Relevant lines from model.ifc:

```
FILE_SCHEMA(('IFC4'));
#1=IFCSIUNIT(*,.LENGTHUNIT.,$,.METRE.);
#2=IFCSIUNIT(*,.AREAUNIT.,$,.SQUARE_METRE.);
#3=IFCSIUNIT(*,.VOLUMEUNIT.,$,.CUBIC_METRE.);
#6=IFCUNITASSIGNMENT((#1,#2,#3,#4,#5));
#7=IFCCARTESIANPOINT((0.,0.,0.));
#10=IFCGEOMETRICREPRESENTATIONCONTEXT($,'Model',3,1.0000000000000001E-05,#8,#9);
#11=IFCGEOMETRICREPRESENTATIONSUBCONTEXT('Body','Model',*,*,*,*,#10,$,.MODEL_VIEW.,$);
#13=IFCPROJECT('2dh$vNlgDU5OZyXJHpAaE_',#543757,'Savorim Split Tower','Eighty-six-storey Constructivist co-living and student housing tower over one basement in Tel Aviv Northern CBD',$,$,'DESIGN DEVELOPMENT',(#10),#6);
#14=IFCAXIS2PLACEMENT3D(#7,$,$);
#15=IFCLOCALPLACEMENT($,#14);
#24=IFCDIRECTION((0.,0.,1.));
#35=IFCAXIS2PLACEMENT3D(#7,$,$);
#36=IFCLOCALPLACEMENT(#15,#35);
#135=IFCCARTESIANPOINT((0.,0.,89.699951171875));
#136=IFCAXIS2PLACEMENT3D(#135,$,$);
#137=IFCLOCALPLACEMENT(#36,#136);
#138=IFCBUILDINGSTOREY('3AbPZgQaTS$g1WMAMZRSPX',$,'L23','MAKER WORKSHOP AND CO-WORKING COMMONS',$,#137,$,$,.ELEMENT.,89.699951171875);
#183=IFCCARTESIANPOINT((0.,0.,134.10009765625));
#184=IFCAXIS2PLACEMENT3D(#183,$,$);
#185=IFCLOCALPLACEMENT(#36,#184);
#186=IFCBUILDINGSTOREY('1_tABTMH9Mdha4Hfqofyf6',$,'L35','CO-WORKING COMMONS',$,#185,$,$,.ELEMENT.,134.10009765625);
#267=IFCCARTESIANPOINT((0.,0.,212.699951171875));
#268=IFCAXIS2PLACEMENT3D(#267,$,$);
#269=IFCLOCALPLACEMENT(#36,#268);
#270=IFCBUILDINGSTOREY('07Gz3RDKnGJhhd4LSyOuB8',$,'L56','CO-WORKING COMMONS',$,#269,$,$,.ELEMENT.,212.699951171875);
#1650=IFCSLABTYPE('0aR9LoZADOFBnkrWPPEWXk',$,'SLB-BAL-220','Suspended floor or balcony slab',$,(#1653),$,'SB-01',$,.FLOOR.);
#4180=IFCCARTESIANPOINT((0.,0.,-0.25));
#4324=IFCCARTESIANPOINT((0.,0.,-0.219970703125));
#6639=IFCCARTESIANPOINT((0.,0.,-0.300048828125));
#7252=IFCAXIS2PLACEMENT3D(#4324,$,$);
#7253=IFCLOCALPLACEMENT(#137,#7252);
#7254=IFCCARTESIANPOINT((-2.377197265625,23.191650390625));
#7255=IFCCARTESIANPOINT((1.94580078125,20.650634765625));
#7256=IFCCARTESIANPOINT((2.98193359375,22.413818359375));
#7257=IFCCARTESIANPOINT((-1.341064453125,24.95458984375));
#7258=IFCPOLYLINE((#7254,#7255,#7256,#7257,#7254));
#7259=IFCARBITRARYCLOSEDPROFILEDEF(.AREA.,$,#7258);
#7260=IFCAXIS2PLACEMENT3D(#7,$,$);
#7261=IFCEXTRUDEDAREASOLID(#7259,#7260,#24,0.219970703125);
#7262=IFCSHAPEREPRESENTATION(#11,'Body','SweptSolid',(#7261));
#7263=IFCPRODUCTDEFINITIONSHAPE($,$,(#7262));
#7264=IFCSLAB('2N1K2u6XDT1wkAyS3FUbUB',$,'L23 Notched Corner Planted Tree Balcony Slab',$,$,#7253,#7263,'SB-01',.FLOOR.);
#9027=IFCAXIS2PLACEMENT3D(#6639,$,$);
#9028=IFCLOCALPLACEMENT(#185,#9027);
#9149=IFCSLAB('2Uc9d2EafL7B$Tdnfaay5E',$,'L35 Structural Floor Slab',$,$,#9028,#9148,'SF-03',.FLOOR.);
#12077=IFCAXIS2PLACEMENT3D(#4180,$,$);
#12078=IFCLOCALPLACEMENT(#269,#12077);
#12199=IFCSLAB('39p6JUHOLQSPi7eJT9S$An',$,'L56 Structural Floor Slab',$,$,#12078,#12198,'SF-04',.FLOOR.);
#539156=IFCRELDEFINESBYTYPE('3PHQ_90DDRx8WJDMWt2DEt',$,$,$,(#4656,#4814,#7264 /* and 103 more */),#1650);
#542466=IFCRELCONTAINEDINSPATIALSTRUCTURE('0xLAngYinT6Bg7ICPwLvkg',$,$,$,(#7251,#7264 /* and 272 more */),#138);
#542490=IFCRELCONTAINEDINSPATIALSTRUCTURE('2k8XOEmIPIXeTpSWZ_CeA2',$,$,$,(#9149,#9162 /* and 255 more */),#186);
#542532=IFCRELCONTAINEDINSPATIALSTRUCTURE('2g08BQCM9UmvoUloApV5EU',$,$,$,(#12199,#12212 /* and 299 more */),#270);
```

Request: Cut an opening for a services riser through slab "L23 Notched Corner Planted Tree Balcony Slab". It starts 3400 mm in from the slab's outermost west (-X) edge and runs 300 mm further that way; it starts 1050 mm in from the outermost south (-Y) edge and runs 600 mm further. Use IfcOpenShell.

```python
import numpy as np
import ifcopenshell
import ifcopenshell.api.feature
import ifcopenshell.api.geometry
import ifcopenshell.api.root
import ifcopenshell.geom
import ifcopenshell.util.placement
import ifcopenshell.util.representation
import ifcopenshell.util.shape
import ifcopenshell.util.unit

model = ifcopenshell.open("model.ifc")
unit_scale = ifcopenshell.util.unit.calculate_unit_scale(model)
settings = ifcopenshell.geom.settings()


def volume(element):
    """Net volume in cubic metres, openings subtracted."""
    shape = ifcopenshell.geom.create_shape(settings, element)
    return ifcopenshell.util.shape.get_volume(shape.geometry)


slab = model.by_id(7264)
before = volume(slab)

# Extent in the slab's own axes, in metres. The edges named are its -X and -Y sides.
slab_shape = ifcopenshell.geom.create_shape(settings, slab)
vertices = ifcopenshell.util.shape.get_vertices(slab_shape.geometry)
x_min, y_min, bottom = vertices.min(axis=0)
top = vertices[:, 2].max()

opening = ifcopenshell.api.root.create_entity(model, ifc_class="IfcOpeningElement", name="Services riser opening", predefined_type="OPENING")
context = ifcopenshell.util.representation.get_context(model, "Model", "Body", "MODEL_VIEW")
width, depth = 0.3, 0.6
outline = [(0.0, 0.0), (width, 0.0), (width, depth), (0.0, depth), (0.0, 0.0)]
# Overshoot both faces by 50 mm so the cut is clean.
shape = ifcopenshell.api.geometry.add_slab_representation(
    model, context=context, depth=top - bottom + 0.1, polyline=outline
)
ifcopenshell.api.geometry.assign_representation(model, product=opening, representation=shape)

matrix = ifcopenshell.util.placement.get_local_placement(slab.ObjectPlacement)
matrix[:, 3] = matrix @ np.append(np.array([x_min + 3.4, y_min + 1.05, bottom - 0.05]) / unit_scale, 1.0)
ifcopenshell.api.geometry.edit_object_placement(model, product=opening, matrix=matrix, is_si=False)
ifcopenshell.api.feature.add_feature(model, feature=opening, element=slab)

after = volume(slab)

print(f"slab volume {before:.3f} -> {after:.3f} m3")

model.write("model_updated.ifc")
```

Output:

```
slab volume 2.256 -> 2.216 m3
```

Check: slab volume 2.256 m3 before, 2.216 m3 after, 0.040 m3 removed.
